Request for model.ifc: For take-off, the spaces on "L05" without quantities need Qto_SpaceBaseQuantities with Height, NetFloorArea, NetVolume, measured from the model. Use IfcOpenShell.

First a look at what the model holds.

```python
import ifcopenshell
import ifcopenshell.util.element
import ifcopenshell.util.unit

model = ifcopenshell.open("model.ifc")
print(model.schema)
for unit_type in ("LENGTHUNIT", "AREAUNIT", "VOLUMEUNIT"):
    print(unit_type, ifcopenshell.util.unit.calculate_unit_scale(model, unit_type))
storey = next(s for s in model.by_type("IfcBuildingStorey") if s.Name == "L05")
spaces = [e for e in ifcopenshell.util.element.get_decomposition(storey) if e.is_a("IfcSpace")]
for e in sorted(spaces, key=lambda e: e.id()):
    print(e.id(), e.is_a(), e.Name, list(ifcopenshell.util.element.get_psets(e, qtos_only=True)), sep=" | ")
```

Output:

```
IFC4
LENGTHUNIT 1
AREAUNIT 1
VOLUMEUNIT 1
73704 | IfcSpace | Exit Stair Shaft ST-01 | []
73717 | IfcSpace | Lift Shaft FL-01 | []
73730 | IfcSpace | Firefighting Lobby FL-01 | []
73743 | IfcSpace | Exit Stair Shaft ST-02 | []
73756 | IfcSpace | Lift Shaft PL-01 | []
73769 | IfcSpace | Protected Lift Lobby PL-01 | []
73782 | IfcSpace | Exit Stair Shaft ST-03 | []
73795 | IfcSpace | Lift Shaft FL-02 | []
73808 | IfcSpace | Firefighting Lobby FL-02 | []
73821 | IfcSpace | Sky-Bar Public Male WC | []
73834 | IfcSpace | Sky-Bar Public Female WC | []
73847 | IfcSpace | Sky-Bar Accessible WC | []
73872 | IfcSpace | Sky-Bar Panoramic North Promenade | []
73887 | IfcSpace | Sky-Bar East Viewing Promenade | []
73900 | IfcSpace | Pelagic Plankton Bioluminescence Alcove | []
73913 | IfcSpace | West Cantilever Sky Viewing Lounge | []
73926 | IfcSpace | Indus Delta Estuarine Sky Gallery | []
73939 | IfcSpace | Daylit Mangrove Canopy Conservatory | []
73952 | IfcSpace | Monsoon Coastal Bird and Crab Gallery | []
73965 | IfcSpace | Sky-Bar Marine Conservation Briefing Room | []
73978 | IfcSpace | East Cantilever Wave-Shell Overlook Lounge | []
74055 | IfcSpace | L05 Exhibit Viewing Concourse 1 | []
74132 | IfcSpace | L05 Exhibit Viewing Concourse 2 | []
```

```python
import ifcopenshell
import ifcopenshell.api.pset
import ifcopenshell.geom
import ifcopenshell.util.element
import ifcopenshell.util.shape
import ifcopenshell.util.unit

model = ifcopenshell.open("model.ifc")
unit_scale = ifcopenshell.util.unit.calculate_unit_scale(model)
area_scale = ifcopenshell.util.unit.calculate_unit_scale(model, "AREAUNIT")
volume_scale = ifcopenshell.util.unit.calculate_unit_scale(model, "VOLUMEUNIT")
settings = ifcopenshell.geom.settings()

storey = next(s for s in model.by_type("IfcBuildingStorey") if s.Name == "L05")
spaces = [e for e in ifcopenshell.util.element.get_decomposition(storey) if e.is_a("IfcSpace")]

for e in sorted(spaces, key=lambda e: e.id()):
    if ifcopenshell.util.element.get_psets(e, qtos_only=True, should_inherit=False):
        continue
    # Geometry comes back in metres, in the element's own axes.
    shape = ifcopenshell.geom.create_shape(settings, e)
    values = {
        "Height": ifcopenshell.util.shape.get_z(shape.geometry) / unit_scale,
        "NetFloorArea": ifcopenshell.util.shape.get_footprint_area(shape.geometry) / area_scale,
        "NetVolume": ifcopenshell.util.shape.get_volume(shape.geometry) / volume_scale,
    }
    qto = ifcopenshell.api.pset.add_qto(model, product=e, name="Qto_SpaceBaseQuantities")
    ifcopenshell.api.pset.edit_qto(model, qto=qto, properties=values)
    print(e.id(), {k: round(v, 3) for k, v in values.items()})

model.write("model_rev.ifc")
```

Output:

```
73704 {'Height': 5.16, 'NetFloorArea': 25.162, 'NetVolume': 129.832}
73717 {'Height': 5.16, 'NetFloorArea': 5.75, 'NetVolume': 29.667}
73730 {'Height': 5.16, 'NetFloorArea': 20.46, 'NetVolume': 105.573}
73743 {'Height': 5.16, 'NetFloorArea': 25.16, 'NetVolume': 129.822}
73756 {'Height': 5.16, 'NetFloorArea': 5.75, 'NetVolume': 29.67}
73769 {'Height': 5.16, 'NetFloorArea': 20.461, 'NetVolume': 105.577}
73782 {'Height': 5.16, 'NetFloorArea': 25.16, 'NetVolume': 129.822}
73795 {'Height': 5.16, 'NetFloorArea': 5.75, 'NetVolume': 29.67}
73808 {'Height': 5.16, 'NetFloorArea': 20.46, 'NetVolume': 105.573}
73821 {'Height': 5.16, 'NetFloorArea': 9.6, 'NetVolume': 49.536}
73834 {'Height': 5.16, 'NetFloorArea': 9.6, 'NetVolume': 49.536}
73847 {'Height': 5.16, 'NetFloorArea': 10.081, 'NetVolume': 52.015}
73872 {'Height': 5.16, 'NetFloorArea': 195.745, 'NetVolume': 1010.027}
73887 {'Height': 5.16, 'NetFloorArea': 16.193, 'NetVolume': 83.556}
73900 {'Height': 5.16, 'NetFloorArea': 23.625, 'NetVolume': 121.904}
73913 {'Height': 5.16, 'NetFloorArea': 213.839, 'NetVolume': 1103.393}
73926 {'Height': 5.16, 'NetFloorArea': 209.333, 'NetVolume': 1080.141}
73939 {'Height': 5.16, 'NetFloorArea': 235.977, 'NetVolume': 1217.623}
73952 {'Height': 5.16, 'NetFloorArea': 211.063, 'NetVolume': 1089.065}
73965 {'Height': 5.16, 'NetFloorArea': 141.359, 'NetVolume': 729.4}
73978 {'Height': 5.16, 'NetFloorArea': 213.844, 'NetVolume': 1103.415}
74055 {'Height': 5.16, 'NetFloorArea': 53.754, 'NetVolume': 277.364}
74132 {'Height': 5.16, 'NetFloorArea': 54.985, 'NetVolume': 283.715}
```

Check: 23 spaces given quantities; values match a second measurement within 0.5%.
